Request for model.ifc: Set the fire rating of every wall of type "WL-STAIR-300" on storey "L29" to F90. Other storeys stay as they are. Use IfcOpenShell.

First a look at what the model holds.

```python
import ifcopenshell
import ifcopenshell.util.element

model = ifcopenshell.open("model.ifc")
print(model.schema)
storey = next(s for s in model.by_type("IfcBuildingStorey") if s.Name == "L29")
walls = [e for e in ifcopenshell.util.element.get_decomposition(storey) if e.is_a("IfcWall")]
seen = {}
for e in walls:
    element_type = ifcopenshell.util.element.get_type(e)
    key = (element_type.Name if element_type != e and element_type else None, ifcopenshell.util.element.get_pset(e, "Pset_WallCommon", "FireRating"))
    seen[key] = seen.get(key, 0) + 1
for (name, value), count in sorted(seen.items(), key=str):
    print(count, "x", name, "|", value)
```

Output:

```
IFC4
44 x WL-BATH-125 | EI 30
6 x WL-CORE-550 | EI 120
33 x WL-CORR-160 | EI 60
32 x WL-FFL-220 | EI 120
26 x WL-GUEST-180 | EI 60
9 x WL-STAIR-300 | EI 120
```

```python
import ifcopenshell
import ifcopenshell.api.pset
import ifcopenshell.util.element

model = ifcopenshell.open("model.ifc")

storey = next(s for s in model.by_type("IfcBuildingStorey") if s.Name == "L29")
walls = [e for e in ifcopenshell.util.element.get_decomposition(storey) if e.is_a("IfcWall")]

count = 0
for e in walls:
    element_type = ifcopenshell.util.element.get_type(e)
    if element_type in (None, e) or element_type.Name != "WL-STAIR-300":
        continue
    # add_pset returns the element's existing set when there is one.
    pset = ifcopenshell.api.pset.add_pset(model, product=e, name="Pset_WallCommon")
    ifcopenshell.api.pset.edit_pset(model, pset=pset, properties={"FireRating": "F90"})
    count += 1

print(count, "walls updated")

model.write("model_rev.ifc")
```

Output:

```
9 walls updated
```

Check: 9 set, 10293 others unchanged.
